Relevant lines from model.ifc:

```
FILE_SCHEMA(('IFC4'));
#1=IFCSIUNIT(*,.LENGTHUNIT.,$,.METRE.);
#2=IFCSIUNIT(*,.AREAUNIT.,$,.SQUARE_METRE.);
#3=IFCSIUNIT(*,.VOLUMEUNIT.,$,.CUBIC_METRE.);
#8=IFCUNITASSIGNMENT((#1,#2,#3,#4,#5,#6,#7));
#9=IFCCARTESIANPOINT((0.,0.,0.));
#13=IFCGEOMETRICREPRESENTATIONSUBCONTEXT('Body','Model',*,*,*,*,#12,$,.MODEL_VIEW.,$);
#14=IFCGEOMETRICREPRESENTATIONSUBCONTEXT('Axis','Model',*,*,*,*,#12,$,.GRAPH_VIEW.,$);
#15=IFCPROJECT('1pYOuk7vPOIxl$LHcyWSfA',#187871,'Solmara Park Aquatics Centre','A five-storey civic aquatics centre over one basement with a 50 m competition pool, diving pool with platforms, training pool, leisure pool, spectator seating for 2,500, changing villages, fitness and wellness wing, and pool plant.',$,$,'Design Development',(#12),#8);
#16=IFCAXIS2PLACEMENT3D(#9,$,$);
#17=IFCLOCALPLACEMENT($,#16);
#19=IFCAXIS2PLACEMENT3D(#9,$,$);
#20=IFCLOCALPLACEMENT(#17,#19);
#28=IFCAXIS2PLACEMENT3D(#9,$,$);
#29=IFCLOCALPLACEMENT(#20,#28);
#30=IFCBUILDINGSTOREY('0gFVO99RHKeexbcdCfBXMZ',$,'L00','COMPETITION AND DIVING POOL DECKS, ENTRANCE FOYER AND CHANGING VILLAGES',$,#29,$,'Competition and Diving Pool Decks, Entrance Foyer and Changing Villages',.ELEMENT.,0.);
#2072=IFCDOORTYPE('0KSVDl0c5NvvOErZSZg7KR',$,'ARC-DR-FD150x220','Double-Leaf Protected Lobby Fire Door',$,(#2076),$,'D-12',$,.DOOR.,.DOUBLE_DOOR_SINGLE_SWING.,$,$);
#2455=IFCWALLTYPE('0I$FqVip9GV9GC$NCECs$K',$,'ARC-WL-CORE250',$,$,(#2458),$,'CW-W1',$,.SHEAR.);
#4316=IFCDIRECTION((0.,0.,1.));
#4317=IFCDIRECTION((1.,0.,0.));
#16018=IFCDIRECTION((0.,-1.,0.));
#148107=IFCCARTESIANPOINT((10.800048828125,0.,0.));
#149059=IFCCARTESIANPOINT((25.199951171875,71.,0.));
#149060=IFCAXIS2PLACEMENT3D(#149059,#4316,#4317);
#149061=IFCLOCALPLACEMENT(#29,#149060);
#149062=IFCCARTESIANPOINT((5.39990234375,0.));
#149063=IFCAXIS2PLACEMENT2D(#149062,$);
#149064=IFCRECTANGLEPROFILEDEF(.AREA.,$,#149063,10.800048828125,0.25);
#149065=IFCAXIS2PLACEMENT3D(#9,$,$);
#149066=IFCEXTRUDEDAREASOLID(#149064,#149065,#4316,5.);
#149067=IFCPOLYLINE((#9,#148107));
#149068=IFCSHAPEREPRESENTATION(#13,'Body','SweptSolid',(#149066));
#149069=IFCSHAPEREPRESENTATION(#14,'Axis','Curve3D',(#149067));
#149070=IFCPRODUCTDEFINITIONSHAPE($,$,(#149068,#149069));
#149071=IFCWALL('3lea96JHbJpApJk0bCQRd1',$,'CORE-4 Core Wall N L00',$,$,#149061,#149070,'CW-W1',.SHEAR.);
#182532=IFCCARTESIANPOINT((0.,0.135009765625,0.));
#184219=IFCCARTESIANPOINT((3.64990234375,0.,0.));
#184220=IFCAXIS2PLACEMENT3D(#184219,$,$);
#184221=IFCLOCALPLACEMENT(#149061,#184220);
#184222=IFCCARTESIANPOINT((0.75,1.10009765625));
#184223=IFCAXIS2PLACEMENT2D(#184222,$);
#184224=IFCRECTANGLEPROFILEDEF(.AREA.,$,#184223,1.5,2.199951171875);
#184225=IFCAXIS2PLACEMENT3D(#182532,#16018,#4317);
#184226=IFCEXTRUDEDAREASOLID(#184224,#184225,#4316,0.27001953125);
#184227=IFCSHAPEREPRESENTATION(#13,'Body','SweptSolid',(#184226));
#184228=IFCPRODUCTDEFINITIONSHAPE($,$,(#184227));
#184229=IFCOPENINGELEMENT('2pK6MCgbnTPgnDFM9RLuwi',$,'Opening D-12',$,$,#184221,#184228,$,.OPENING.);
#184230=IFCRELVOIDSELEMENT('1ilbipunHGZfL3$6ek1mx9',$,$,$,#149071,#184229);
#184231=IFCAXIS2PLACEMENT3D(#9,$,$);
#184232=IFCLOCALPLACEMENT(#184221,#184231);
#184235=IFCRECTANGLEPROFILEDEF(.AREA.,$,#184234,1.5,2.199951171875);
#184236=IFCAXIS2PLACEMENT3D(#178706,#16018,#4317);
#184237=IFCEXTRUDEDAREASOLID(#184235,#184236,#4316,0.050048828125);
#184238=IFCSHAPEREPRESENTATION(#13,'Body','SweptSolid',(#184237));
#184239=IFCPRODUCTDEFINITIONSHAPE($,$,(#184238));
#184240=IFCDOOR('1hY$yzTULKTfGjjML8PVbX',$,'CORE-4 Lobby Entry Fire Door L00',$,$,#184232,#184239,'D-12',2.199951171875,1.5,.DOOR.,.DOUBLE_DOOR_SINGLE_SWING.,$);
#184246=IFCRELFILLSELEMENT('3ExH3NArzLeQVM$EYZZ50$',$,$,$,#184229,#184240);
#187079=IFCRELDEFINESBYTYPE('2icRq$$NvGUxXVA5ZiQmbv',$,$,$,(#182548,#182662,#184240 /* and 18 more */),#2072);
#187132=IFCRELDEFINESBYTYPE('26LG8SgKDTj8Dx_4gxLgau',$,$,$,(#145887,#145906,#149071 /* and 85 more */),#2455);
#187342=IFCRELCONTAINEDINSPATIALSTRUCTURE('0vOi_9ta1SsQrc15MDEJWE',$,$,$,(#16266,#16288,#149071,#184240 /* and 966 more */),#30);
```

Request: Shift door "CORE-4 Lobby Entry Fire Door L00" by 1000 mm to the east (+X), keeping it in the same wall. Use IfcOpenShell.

```python
import ifcopenshell
import ifcopenshell.api.geometry
import ifcopenshell.util.placement
import ifcopenshell.util.unit

model = ifcopenshell.open("model.ifc")
unit_scale = ifcopenshell.util.unit.calculate_unit_scale(model)

door = model.by_guid("1hY$yzTULKTfGjjML8PVbX")
opening = door.FillsVoids[0].RelatingOpeningElement
wall = opening.VoidsElements[0].RelatingBuildingElement

wall_matrix = ifcopenshell.util.placement.get_local_placement(wall.ObjectPlacement)
shift = wall_matrix[:3, 0] * 1 / unit_scale
before = ifcopenshell.util.placement.get_local_placement(door.ObjectPlacement)[:3, 3].copy()

# The door is placed relative to its opening, so it follows when the opening moves.
matrix = ifcopenshell.util.placement.get_local_placement(opening.ObjectPlacement)
matrix[:3, 3] += shift
ifcopenshell.api.geometry.edit_object_placement(
    model, product=opening, matrix=matrix, is_si=False, should_transform_children=True
)

after = ifcopenshell.util.placement.get_local_placement(door.ObjectPlacement)[:3, 3]
print("door moved by", (after - before).round(3) + 0.0)

model.write("model_edited.ifc")
```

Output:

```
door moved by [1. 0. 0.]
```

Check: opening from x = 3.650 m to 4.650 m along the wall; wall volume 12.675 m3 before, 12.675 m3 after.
